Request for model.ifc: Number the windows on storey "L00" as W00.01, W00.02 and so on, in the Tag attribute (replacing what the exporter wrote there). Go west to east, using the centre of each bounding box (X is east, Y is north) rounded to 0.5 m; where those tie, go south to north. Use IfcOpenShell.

First a look at what the model holds.

```python
import ifcopenshell
import ifcopenshell.util.element
import ifcopenshell.util.placement

model = ifcopenshell.open("model.ifc")
print(model.schema)
storey = next(s for s in model.by_type("IfcBuildingStorey") if s.Name == "L00")
windows = [e for e in ifcopenshell.util.element.get_decomposition(storey) if e.is_a("IfcWindow")]
for e in sorted(windows, key=lambda e: e.id()):
    origin = ifcopenshell.util.placement.get_local_placement(e.ObjectPlacement)[:3, 3]
    print(e.id(), e.Tag, e.Name, origin.round(2) + 0.0, sep=" | ")
```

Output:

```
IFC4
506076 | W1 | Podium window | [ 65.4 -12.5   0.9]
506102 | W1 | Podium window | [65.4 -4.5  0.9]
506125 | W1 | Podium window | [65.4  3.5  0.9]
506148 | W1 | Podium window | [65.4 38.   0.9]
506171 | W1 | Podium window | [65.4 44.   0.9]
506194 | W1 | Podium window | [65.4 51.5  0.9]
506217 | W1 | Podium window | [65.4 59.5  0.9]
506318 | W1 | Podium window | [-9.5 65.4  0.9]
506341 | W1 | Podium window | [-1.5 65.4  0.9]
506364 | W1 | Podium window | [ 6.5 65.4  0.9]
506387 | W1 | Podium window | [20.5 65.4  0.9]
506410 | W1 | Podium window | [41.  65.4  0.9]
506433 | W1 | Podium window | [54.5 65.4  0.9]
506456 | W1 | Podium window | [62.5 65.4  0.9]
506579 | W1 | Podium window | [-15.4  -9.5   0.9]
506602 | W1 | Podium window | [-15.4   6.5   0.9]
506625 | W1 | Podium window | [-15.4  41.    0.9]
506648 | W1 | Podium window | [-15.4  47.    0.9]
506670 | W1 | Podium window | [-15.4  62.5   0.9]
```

```python
import ifcopenshell
import ifcopenshell.geom
import ifcopenshell.util.element
import ifcopenshell.util.shape

model = ifcopenshell.open("model.ifc")
settings = ifcopenshell.geom.settings()
settings.set("use-world-coords", True)


def centre(element):
    shape = ifcopenshell.geom.create_shape(settings, element)
    return ifcopenshell.util.shape.get_bbox_centroid(shape.geometry)


storey = next(s for s in model.by_type("IfcBuildingStorey") if s.Name == "L00")
windows = [e for e in ifcopenshell.util.element.get_decomposition(storey) if e.is_a("IfcWindow")]

# Insertion points can sit at a corner or the storey origin, so sort by the geometry (in metres).
centres = {e: centre(e) for e in windows}
windows.sort(key=lambda e: (round(centres[e][0] / 0.5), centres[e][1]))

for i, e in enumerate(windows, start=1):
    number = f"W00.{i:02d}"
    e.Tag = number
    print(e.id(), number)

model.write("model_rev.ifc")
```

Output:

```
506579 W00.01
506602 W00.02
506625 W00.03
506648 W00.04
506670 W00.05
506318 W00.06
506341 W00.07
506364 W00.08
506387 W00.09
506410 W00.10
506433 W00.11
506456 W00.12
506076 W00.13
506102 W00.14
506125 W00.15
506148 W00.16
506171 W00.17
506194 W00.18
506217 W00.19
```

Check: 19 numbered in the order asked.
